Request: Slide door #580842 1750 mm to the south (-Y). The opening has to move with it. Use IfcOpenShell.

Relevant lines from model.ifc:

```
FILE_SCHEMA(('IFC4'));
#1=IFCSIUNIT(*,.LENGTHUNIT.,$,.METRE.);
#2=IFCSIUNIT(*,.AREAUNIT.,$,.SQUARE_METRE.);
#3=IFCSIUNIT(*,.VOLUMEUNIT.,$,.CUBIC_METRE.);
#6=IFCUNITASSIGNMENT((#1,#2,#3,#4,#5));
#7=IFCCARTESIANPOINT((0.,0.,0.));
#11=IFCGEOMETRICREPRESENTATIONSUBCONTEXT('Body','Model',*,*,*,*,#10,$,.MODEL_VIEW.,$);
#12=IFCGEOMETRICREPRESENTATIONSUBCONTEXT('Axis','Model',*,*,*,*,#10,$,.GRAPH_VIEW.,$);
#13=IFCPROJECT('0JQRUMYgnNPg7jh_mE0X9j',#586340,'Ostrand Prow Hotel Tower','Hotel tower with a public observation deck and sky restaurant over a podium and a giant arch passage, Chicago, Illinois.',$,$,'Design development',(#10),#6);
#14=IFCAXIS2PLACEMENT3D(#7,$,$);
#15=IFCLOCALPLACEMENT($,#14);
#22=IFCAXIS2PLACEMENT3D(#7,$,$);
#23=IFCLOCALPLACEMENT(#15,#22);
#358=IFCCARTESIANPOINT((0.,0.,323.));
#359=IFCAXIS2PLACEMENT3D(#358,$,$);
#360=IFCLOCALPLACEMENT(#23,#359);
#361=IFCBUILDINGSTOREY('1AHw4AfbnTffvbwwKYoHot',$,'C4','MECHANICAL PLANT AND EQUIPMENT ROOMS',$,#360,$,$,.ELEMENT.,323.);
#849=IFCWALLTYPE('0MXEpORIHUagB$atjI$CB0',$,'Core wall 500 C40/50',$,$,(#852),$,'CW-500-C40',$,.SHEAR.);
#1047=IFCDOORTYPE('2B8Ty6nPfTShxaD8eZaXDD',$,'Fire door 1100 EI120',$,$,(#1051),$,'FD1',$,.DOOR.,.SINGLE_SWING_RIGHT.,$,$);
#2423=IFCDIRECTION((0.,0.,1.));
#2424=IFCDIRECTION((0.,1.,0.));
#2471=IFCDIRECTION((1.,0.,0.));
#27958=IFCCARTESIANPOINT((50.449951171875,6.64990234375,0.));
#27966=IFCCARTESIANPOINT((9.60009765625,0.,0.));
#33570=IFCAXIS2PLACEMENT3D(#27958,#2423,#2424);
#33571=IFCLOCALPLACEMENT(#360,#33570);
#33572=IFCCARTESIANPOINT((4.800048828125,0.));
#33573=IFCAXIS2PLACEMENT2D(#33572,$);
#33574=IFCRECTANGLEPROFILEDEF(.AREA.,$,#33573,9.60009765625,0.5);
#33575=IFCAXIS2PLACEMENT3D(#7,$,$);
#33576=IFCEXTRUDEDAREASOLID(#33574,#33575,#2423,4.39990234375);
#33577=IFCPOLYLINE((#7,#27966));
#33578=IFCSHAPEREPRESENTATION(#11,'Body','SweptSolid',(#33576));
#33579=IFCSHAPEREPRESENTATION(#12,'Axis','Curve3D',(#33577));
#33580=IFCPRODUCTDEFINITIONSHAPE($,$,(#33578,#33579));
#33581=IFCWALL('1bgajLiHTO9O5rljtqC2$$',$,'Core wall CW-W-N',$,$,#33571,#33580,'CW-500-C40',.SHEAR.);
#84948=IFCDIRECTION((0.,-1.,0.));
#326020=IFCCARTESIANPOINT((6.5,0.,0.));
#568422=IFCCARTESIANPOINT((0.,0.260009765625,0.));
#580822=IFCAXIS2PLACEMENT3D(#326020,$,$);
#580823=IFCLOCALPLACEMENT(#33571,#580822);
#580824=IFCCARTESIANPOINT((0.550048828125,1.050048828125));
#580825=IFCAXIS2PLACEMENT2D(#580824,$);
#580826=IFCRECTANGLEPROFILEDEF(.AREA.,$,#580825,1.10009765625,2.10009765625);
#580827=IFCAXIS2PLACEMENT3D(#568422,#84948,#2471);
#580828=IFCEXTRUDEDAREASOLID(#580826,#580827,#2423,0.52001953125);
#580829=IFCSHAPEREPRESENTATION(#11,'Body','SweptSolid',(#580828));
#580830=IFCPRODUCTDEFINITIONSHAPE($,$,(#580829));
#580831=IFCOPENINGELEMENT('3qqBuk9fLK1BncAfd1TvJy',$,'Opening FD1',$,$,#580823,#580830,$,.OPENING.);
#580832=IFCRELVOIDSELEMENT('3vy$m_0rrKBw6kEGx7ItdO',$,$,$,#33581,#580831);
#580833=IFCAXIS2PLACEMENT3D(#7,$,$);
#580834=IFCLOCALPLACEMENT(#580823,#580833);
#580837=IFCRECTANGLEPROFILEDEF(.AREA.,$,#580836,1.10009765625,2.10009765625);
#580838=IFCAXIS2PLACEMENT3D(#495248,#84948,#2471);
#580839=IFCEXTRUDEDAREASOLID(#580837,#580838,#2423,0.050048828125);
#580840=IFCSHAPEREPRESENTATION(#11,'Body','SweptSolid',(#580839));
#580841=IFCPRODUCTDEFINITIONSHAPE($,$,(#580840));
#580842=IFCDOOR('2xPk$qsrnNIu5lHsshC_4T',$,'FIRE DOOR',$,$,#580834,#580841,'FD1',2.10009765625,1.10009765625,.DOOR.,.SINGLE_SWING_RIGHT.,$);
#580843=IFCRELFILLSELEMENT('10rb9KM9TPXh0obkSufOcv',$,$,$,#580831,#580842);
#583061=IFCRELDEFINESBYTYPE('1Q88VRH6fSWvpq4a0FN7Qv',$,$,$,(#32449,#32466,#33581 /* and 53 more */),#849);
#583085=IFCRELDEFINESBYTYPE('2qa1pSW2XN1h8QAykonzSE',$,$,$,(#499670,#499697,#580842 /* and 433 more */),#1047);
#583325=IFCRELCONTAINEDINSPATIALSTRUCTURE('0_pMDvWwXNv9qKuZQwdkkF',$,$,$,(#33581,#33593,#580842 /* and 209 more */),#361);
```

```python
import ifcopenshell
import ifcopenshell.api.geometry
import ifcopenshell.util.placement
import ifcopenshell.util.unit

model = ifcopenshell.open("model.ifc")
unit_scale = ifcopenshell.util.unit.calculate_unit_scale(model)

door = model.by_guid("2xPk$qsrnNIu5lHsshC_4T")
opening = door.FillsVoids[0].RelatingOpeningElement
wall = opening.VoidsElements[0].RelatingBuildingElement

wall_matrix = ifcopenshell.util.placement.get_local_placement(wall.ObjectPlacement)
shift = wall_matrix[:3, 0] * -1.75 / unit_scale
before = ifcopenshell.util.placement.get_local_placement(door.ObjectPlacement)[:3, 3].copy()

# The door is placed relative to its opening, so it follows when the opening moves.
matrix = ifcopenshell.util.placement.get_local_placement(opening.ObjectPlacement)
matrix[:3, 3] += shift
ifcopenshell.api.geometry.edit_object_placement(
    model, product=opening, matrix=matrix, is_si=False, should_transform_children=True
)

after = ifcopenshell.util.placement.get_local_placement(door.ObjectPlacement)[:3, 3]
print("door moved by", (after - before).round(3) + 0.0)

model.write("model_updated.ifc")
```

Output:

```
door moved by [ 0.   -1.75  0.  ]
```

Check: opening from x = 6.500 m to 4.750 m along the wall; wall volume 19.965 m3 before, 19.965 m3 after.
